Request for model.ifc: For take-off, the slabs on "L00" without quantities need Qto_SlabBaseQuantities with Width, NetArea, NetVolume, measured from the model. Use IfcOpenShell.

First a look at what the model holds.

```python
import ifcopenshell
import ifcopenshell.util.element
import ifcopenshell.util.unit

model = ifcopenshell.open("model.ifc")
print(model.schema)
for unit_type in ("LENGTHUNIT", "AREAUNIT", "VOLUMEUNIT"):
    print(unit_type, ifcopenshell.util.unit.calculate_unit_scale(model, unit_type))
storey = next(s for s in model.by_type("IfcBuildingStorey") if s.Name == "L00")
slabs = [e for e in ifcopenshell.util.element.get_decomposition(storey) if e.is_a("IfcSlab")]
for e in sorted(slabs, key=lambda e: e.id()):
    print(e.id(), e.is_a(), e.Name, list(ifcopenshell.util.element.get_psets(e, qtos_only=True)), sep=" | ")
```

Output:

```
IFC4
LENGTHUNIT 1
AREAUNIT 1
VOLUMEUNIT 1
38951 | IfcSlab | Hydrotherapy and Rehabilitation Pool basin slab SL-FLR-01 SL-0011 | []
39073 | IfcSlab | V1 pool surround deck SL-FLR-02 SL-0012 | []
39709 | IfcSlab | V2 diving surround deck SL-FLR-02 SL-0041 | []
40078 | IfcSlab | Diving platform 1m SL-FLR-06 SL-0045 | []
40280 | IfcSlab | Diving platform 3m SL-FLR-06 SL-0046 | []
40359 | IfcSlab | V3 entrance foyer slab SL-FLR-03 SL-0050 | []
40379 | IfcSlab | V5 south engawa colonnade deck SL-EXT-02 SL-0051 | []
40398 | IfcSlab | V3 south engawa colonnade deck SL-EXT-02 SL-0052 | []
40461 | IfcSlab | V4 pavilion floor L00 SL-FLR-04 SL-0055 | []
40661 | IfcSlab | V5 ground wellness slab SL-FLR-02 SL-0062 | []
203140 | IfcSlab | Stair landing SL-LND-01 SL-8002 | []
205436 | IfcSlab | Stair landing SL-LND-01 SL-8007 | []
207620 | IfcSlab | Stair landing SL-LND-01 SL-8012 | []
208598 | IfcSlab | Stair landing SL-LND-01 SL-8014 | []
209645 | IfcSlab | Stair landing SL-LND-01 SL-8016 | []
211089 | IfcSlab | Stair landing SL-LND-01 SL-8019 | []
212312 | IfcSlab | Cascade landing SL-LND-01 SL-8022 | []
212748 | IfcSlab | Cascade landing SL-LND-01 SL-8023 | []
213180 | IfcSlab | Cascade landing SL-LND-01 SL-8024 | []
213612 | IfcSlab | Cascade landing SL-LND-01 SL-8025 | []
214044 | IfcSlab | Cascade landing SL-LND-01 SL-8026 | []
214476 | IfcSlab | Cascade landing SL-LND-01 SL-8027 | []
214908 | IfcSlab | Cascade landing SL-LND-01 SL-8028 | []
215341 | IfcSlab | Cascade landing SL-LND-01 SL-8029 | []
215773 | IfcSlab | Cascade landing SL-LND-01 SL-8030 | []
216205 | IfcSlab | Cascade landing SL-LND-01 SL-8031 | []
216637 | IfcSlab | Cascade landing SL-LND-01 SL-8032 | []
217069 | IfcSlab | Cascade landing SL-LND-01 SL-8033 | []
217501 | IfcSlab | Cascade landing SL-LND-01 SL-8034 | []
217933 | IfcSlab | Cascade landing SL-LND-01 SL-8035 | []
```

```python
import ifcopenshell
import ifcopenshell.api.pset
import ifcopenshell.geom
import ifcopenshell.util.element
import ifcopenshell.util.shape
import ifcopenshell.util.unit

model = ifcopenshell.open("model.ifc")
unit_scale = ifcopenshell.util.unit.calculate_unit_scale(model)
area_scale = ifcopenshell.util.unit.calculate_unit_scale(model, "AREAUNIT")
volume_scale = ifcopenshell.util.unit.calculate_unit_scale(model, "VOLUMEUNIT")
settings = ifcopenshell.geom.settings()

storey = next(s for s in model.by_type("IfcBuildingStorey") if s.Name == "L00")
slabs = [e for e in ifcopenshell.util.element.get_decomposition(storey) if e.is_a("IfcSlab")]

for e in sorted(slabs, key=lambda e: e.id()):
    if ifcopenshell.util.element.get_psets(e, qtos_only=True, should_inherit=False):
        continue
    # Geometry comes back in metres, in the element's own axes.
    shape = ifcopenshell.geom.create_shape(settings, e)
    values = {
        "Width": ifcopenshell.util.shape.get_z(shape.geometry) / unit_scale,
        "NetArea": ifcopenshell.util.shape.get_footprint_area(shape.geometry) / area_scale,
        "NetVolume": ifcopenshell.util.shape.get_volume(shape.geometry) / volume_scale,
    }
    qto = ifcopenshell.api.pset.add_qto(model, product=e, name="Qto_SlabBaseQuantities")
    ifcopenshell.api.pset.edit_qto(model, qto=qto, properties=values)
    print(e.id(), {k: round(v, 3) for k, v in values.items()})

model.write("model_edited.ifc")
```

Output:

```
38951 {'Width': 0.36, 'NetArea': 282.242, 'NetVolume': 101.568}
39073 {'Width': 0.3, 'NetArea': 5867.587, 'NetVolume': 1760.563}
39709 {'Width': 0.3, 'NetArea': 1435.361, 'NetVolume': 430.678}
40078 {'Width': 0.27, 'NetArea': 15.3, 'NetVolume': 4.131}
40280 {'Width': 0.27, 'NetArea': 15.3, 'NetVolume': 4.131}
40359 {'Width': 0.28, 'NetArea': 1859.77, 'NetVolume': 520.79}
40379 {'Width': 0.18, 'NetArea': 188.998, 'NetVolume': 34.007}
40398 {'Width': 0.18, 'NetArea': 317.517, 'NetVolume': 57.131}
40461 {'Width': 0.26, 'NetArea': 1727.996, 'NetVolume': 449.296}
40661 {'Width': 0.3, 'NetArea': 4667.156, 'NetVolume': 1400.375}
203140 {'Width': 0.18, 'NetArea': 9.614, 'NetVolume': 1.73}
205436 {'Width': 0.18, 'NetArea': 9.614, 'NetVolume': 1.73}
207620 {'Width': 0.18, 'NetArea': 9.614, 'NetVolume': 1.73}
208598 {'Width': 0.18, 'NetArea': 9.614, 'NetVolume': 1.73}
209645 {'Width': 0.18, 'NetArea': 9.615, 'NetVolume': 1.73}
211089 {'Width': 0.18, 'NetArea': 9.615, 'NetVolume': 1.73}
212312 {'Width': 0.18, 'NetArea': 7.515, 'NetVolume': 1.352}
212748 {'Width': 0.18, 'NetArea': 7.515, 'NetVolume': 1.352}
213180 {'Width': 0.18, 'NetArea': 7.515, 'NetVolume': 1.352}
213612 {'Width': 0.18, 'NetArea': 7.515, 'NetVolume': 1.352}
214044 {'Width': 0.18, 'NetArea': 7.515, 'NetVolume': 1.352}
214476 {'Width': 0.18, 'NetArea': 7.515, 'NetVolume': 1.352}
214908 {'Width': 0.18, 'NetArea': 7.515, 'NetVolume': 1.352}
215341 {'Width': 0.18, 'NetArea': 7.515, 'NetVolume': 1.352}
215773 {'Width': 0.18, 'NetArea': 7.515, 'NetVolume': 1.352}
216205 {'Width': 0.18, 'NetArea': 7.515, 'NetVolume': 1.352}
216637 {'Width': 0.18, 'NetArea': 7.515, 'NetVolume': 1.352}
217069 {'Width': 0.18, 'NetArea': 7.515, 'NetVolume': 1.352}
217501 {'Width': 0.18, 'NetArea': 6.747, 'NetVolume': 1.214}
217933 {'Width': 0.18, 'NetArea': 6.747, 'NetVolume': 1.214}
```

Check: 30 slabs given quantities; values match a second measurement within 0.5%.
